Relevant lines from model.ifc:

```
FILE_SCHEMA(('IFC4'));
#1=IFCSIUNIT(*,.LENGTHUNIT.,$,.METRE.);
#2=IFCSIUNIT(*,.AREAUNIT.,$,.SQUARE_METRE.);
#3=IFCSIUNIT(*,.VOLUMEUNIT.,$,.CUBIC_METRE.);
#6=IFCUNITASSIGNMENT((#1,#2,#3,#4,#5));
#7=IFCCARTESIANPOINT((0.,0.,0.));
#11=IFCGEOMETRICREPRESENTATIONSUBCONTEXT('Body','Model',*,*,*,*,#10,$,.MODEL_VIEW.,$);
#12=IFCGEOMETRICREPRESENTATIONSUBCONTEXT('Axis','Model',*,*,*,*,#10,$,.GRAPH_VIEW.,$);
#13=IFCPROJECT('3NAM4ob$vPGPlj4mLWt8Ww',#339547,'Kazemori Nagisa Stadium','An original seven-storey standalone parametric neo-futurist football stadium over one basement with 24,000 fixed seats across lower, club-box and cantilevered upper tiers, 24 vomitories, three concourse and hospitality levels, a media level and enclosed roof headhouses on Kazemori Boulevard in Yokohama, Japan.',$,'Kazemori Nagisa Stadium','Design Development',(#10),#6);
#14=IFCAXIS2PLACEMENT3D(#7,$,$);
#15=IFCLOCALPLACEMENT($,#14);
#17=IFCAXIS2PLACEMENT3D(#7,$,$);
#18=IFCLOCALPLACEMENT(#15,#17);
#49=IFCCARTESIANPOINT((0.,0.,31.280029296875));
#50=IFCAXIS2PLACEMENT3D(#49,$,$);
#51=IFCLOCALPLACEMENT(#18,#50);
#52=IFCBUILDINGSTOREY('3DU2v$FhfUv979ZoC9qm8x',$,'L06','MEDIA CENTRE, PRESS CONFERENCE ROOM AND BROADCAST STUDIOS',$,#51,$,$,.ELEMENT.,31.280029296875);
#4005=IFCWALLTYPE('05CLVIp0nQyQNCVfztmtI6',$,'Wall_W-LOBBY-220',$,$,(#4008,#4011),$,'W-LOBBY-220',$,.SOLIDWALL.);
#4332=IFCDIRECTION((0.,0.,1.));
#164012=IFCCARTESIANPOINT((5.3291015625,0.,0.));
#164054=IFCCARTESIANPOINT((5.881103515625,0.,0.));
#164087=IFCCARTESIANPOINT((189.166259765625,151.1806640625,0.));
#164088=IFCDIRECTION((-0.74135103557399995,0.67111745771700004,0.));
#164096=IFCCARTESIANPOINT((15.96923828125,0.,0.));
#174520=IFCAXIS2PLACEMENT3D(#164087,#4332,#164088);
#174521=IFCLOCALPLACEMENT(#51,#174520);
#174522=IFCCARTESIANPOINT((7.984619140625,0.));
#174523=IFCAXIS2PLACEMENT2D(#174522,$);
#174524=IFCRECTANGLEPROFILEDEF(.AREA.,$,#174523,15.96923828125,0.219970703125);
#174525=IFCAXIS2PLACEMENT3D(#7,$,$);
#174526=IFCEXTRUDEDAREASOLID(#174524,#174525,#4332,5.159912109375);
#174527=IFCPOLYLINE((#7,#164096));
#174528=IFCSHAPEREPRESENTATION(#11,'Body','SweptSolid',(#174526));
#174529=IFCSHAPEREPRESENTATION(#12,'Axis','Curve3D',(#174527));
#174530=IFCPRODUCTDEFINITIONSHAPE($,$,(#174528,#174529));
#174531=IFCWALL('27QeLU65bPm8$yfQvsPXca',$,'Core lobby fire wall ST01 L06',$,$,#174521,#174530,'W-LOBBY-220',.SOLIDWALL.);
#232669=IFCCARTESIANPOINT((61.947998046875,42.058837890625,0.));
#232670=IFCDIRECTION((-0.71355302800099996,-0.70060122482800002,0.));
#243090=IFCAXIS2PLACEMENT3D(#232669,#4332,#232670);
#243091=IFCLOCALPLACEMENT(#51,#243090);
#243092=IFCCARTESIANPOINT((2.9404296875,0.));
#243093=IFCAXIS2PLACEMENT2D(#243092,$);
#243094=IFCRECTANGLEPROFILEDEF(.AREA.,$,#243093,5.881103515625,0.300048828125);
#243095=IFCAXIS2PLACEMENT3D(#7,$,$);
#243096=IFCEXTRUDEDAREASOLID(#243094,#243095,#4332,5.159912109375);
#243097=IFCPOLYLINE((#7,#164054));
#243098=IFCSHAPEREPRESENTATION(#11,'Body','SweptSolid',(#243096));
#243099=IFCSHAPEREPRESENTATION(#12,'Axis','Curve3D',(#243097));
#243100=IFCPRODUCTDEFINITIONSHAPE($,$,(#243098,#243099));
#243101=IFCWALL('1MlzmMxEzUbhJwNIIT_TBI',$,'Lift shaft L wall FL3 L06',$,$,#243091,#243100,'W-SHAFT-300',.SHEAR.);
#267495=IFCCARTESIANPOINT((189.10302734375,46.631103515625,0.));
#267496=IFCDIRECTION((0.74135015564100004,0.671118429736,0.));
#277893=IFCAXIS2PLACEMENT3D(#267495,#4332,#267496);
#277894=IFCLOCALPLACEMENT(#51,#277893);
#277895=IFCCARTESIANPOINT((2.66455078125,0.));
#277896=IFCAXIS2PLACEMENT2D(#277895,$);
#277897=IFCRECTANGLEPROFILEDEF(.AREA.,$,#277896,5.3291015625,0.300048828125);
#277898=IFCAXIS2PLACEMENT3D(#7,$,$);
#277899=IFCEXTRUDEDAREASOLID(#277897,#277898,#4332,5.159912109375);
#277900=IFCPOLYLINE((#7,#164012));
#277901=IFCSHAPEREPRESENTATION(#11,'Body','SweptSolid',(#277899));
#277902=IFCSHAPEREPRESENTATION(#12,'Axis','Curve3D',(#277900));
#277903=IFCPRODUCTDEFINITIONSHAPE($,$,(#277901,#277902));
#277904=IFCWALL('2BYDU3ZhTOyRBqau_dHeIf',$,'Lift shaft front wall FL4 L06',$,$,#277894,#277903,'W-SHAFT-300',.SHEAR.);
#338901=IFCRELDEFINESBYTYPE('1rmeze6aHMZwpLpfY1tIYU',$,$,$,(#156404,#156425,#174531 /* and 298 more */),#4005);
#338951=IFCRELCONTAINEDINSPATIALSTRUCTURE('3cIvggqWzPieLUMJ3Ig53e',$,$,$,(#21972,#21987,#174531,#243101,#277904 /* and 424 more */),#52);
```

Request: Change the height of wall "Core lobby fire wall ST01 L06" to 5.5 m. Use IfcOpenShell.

```python
import ifcopenshell
import ifcopenshell.geom
import ifcopenshell.util.representation
import ifcopenshell.util.shape
import ifcopenshell.util.unit

model = ifcopenshell.open("model.ifc")
unit_scale = ifcopenshell.util.unit.calculate_unit_scale(model)
settings = ifcopenshell.geom.settings()


def volume(element):
    """Net volume in cubic metres, openings subtracted."""
    shape = ifcopenshell.geom.create_shape(settings, element)
    return ifcopenshell.util.shape.get_volume(shape.geometry)


wall = model.by_id(174531)
before = volume(wall)

body = ifcopenshell.util.representation.get_representation(wall, "Model", "Body")
solid = body.Items[0]
old_height = solid.Depth
solid.Depth = 5.5 / unit_scale
after = volume(wall)

print(f"height {old_height:g} -> {solid.Depth:g}, volume {before:.3f} -> {after:.3f} m3")

model.write("model-out.ifc")
```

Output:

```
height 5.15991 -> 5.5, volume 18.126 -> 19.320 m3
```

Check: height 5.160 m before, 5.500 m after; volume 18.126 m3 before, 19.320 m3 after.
